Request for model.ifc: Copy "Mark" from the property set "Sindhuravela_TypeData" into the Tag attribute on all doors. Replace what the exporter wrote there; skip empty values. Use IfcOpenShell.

First a look at what the model holds.

```python
import ifcopenshell
import ifcopenshell.util.element

model = ifcopenshell.open("model.ifc")
print(model.schema)
doors = model.by_type("IfcDoor")
print(len(doors), "doors")
for e in doors[:8]:
    source = ifcopenshell.util.element.get_pset(e, "Sindhuravela_TypeData", "Mark")
    target = e.Tag
    print(e.id(), repr(source), repr(target), sep=" | ")
```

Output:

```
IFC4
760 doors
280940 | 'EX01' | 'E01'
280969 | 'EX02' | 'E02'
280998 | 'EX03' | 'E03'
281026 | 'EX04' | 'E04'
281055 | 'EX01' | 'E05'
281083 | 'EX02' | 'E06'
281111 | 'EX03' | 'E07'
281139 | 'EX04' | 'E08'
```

```python
import ifcopenshell
import ifcopenshell.util.element

model = ifcopenshell.open("model.ifc")

count = 0
for e in model.by_type("IfcDoor"):
    value = ifcopenshell.util.element.get_pset(e, "Sindhuravela_TypeData", "Mark")
    current = e.Tag
    if not value or not value.strip() or current == value:
        continue
    e.Tag = value
    count += 1

print(count, "doors updated")

model.write("model_updated.ifc")
```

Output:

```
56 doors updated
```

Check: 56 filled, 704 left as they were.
